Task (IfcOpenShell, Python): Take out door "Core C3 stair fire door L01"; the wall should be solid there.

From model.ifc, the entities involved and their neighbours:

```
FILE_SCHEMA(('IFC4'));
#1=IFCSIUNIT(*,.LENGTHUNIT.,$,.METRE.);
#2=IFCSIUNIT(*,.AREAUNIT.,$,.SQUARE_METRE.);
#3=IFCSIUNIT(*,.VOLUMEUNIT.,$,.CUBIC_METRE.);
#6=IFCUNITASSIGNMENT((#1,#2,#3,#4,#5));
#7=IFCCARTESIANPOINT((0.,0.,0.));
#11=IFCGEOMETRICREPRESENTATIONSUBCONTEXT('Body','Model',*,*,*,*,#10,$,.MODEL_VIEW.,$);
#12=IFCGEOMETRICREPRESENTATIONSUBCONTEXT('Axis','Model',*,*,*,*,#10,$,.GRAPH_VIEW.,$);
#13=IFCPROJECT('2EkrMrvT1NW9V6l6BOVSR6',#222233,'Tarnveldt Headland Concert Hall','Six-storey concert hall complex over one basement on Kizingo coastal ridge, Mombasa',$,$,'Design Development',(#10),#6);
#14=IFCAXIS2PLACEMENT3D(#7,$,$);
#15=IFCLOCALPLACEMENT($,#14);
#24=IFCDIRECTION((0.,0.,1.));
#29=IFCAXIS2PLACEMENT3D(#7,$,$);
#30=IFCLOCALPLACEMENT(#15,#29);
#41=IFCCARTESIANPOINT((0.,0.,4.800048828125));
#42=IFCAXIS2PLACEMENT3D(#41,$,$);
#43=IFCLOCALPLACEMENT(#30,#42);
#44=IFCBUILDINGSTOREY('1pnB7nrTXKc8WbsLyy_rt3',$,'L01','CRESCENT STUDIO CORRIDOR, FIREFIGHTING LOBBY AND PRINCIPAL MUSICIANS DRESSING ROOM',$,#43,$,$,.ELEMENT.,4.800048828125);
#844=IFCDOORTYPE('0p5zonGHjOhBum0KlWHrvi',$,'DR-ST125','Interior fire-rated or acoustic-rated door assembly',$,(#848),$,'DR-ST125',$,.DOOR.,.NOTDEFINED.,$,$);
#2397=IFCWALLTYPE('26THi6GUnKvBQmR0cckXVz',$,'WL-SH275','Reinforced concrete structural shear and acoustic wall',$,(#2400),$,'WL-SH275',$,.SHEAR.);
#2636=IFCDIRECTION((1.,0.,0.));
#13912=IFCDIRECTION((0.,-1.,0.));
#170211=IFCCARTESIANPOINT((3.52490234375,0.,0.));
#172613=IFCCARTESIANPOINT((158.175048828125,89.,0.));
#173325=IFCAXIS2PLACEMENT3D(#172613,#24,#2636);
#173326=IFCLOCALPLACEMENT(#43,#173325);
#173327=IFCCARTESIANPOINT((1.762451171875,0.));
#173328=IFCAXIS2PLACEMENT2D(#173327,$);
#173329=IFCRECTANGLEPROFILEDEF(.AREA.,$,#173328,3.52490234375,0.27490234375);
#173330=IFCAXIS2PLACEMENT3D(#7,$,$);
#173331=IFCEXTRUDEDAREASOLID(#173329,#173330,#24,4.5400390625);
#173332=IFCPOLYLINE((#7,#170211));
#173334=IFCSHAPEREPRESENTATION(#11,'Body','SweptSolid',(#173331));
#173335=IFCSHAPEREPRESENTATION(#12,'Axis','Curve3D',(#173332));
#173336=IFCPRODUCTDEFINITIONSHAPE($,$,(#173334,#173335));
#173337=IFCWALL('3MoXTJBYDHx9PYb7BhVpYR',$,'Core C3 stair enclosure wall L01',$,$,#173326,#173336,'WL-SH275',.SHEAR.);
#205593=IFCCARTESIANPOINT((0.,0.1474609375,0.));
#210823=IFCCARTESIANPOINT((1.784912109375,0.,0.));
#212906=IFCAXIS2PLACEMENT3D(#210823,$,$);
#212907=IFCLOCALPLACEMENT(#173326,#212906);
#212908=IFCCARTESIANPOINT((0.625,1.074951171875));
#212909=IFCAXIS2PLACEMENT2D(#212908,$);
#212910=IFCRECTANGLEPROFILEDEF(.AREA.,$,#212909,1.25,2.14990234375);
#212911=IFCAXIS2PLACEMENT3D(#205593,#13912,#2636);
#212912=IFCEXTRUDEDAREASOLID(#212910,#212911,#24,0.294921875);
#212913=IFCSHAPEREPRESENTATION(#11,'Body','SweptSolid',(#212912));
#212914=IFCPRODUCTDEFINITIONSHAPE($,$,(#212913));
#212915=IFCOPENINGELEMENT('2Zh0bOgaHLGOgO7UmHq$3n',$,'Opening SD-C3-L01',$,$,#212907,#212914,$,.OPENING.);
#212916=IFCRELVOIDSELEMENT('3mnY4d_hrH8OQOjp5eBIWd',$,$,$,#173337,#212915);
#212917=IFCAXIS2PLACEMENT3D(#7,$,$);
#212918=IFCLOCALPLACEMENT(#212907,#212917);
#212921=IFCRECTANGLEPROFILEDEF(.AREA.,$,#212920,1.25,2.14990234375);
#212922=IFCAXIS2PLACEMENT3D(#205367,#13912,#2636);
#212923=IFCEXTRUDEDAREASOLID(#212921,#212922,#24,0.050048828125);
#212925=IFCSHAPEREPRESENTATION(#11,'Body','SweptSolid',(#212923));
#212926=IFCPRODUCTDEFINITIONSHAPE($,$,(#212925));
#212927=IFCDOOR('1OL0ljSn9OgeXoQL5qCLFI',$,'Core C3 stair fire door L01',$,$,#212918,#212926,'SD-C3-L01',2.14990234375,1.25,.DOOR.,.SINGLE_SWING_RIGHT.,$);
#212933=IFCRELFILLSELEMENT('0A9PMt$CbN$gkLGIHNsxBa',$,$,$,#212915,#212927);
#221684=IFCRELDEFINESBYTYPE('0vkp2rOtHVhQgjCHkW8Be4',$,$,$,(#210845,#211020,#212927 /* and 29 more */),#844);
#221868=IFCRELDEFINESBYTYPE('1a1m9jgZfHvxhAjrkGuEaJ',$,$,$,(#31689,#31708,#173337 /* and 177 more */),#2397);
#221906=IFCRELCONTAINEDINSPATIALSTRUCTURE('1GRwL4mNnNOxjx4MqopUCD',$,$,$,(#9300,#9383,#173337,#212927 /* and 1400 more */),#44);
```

```python
import ifcopenshell
import ifcopenshell.api.feature
import ifcopenshell.api.root
import ifcopenshell.geom
import ifcopenshell.util.shape

model = ifcopenshell.open("model.ifc")
settings = ifcopenshell.geom.settings()


def volume(element):
    """Net volume in cubic metres, openings subtracted."""
    shape = ifcopenshell.geom.create_shape(settings, element)
    return ifcopenshell.util.shape.get_volume(shape.geometry)


door = model.by_id(212927)
opening = door.FillsVoids[0].RelatingOpeningElement
wall = opening.VoidsElements[0].RelatingBuildingElement
before = volume(wall)

ifcopenshell.api.root.remove_product(model, product=door)
ifcopenshell.api.feature.remove_feature(model, feature=opening)

after = volume(wall)

print(f"wall volume {before:.3f} -> {after:.3f} m3")

model.write("model-out.ifc")
```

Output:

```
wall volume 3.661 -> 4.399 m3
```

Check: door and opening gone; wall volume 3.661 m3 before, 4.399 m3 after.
